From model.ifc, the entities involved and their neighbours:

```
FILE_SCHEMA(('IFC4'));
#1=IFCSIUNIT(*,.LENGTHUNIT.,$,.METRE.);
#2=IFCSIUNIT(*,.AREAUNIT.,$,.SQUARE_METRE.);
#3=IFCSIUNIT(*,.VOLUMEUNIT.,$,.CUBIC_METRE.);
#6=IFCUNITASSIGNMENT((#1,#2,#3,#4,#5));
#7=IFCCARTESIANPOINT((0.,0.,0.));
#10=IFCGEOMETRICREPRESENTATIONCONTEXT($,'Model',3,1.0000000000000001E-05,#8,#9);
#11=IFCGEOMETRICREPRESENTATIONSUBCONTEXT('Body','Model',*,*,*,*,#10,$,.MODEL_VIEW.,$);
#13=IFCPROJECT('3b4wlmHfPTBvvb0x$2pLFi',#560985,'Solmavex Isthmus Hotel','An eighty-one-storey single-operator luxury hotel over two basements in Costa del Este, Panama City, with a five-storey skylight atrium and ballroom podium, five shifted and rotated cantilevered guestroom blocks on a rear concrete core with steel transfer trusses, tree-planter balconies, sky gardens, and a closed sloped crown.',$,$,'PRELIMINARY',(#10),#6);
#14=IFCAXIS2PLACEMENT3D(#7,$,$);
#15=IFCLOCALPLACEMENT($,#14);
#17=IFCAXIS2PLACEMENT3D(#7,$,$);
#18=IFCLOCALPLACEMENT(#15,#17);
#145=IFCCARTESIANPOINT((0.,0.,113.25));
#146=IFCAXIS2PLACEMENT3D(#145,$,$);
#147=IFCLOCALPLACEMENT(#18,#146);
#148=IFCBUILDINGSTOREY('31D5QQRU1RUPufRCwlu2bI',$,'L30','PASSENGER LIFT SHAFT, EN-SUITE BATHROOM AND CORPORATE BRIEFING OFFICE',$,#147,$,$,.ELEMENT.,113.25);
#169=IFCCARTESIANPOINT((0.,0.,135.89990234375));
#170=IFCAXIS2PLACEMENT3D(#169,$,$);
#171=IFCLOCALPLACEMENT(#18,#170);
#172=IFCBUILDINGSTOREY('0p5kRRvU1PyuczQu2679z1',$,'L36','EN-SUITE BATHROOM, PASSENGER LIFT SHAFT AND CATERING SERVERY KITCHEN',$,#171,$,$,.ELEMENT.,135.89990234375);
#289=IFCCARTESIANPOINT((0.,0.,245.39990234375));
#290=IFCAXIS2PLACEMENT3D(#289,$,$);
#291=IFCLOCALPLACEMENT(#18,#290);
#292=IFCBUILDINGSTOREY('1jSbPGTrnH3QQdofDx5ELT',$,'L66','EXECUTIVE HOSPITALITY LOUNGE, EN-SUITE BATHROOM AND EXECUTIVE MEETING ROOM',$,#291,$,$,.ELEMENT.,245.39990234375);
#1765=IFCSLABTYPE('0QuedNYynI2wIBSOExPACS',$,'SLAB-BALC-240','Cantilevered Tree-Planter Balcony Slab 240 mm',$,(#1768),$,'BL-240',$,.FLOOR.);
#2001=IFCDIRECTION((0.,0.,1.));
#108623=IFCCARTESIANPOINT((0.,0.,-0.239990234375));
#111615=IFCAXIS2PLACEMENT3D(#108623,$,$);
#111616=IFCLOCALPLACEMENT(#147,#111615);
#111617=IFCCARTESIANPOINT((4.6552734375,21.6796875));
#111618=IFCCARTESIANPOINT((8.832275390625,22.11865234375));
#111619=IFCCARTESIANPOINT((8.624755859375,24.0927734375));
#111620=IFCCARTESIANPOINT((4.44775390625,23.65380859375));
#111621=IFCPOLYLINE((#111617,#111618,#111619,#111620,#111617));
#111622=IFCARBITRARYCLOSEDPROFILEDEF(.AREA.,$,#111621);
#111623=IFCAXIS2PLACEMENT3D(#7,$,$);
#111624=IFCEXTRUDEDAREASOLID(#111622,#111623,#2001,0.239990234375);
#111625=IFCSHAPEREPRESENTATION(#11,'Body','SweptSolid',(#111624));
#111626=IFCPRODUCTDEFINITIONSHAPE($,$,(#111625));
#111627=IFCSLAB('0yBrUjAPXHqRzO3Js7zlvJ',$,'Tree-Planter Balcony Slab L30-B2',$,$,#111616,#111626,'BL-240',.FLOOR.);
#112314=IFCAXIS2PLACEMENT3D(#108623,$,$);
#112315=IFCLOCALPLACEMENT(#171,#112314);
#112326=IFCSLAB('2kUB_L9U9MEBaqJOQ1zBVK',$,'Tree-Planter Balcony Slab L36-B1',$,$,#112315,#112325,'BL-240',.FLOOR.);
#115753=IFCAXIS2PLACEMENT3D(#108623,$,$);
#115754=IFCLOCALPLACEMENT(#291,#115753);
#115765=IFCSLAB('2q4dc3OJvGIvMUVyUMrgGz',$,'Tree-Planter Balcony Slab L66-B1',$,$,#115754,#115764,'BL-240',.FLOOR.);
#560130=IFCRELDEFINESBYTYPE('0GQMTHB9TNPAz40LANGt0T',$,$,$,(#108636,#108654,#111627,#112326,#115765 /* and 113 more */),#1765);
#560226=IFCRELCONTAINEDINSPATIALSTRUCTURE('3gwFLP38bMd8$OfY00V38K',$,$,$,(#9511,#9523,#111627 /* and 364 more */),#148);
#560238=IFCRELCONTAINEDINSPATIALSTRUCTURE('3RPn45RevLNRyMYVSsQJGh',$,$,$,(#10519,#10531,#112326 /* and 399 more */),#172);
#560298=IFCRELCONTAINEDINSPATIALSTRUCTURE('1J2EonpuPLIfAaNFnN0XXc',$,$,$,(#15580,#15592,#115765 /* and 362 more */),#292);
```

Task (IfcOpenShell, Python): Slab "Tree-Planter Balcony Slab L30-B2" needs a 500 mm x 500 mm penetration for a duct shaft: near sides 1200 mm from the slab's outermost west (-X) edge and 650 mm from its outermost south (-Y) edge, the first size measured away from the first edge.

```python
import numpy as np
import ifcopenshell
import ifcopenshell.api.feature
import ifcopenshell.api.geometry
import ifcopenshell.api.root
import ifcopenshell.geom
import ifcopenshell.util.placement
import ifcopenshell.util.representation
import ifcopenshell.util.shape
import ifcopenshell.util.unit

model = ifcopenshell.open("model.ifc")
unit_scale = ifcopenshell.util.unit.calculate_unit_scale(model)
settings = ifcopenshell.geom.settings()


def volume(element):
    """Net volume in cubic metres, openings subtracted."""
    shape = ifcopenshell.geom.create_shape(settings, element)
    return ifcopenshell.util.shape.get_volume(shape.geometry)


slab = model.by_guid("0yBrUjAPXHqRzO3Js7zlvJ")
before = volume(slab)

# Extent in the slab's own axes, in metres. The edges named are its -X and -Y sides.
slab_shape = ifcopenshell.geom.create_shape(settings, slab)
vertices = ifcopenshell.util.shape.get_vertices(slab_shape.geometry)
x_min, y_min, bottom = vertices.min(axis=0)
top = vertices[:, 2].max()

opening = ifcopenshell.api.root.create_entity(model, ifc_class="IfcOpeningElement", name="Duct shaft opening", predefined_type="OPENING")
context = ifcopenshell.util.representation.get_context(model, "Model", "Body", "MODEL_VIEW")
width, depth = 0.5, 0.5
outline = [(0.0, 0.0), (width, 0.0), (width, depth), (0.0, depth), (0.0, 0.0)]
# Overshoot both faces by 50 mm so the cut is clean.
shape = ifcopenshell.api.geometry.add_slab_representation(
    model, context=context, depth=top - bottom + 0.1, polyline=outline
)
ifcopenshell.api.geometry.assign_representation(model, product=opening, representation=shape)

matrix = ifcopenshell.util.placement.get_local_placement(slab.ObjectPlacement)
matrix[:, 3] = matrix @ np.append(np.array([x_min + 1.2, y_min + 0.65, bottom - 0.05]) / unit_scale, 1.0)
ifcopenshell.api.geometry.edit_object_placement(model, product=opening, matrix=matrix, is_si=False)
ifcopenshell.api.feature.add_feature(model, feature=opening, element=slab)

after = volume(slab)

print(f"slab volume {before:.3f} -> {after:.3f} m3")

model.write("model_updated.ifc")
```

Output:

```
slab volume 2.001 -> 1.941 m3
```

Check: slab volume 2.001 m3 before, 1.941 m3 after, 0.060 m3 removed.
